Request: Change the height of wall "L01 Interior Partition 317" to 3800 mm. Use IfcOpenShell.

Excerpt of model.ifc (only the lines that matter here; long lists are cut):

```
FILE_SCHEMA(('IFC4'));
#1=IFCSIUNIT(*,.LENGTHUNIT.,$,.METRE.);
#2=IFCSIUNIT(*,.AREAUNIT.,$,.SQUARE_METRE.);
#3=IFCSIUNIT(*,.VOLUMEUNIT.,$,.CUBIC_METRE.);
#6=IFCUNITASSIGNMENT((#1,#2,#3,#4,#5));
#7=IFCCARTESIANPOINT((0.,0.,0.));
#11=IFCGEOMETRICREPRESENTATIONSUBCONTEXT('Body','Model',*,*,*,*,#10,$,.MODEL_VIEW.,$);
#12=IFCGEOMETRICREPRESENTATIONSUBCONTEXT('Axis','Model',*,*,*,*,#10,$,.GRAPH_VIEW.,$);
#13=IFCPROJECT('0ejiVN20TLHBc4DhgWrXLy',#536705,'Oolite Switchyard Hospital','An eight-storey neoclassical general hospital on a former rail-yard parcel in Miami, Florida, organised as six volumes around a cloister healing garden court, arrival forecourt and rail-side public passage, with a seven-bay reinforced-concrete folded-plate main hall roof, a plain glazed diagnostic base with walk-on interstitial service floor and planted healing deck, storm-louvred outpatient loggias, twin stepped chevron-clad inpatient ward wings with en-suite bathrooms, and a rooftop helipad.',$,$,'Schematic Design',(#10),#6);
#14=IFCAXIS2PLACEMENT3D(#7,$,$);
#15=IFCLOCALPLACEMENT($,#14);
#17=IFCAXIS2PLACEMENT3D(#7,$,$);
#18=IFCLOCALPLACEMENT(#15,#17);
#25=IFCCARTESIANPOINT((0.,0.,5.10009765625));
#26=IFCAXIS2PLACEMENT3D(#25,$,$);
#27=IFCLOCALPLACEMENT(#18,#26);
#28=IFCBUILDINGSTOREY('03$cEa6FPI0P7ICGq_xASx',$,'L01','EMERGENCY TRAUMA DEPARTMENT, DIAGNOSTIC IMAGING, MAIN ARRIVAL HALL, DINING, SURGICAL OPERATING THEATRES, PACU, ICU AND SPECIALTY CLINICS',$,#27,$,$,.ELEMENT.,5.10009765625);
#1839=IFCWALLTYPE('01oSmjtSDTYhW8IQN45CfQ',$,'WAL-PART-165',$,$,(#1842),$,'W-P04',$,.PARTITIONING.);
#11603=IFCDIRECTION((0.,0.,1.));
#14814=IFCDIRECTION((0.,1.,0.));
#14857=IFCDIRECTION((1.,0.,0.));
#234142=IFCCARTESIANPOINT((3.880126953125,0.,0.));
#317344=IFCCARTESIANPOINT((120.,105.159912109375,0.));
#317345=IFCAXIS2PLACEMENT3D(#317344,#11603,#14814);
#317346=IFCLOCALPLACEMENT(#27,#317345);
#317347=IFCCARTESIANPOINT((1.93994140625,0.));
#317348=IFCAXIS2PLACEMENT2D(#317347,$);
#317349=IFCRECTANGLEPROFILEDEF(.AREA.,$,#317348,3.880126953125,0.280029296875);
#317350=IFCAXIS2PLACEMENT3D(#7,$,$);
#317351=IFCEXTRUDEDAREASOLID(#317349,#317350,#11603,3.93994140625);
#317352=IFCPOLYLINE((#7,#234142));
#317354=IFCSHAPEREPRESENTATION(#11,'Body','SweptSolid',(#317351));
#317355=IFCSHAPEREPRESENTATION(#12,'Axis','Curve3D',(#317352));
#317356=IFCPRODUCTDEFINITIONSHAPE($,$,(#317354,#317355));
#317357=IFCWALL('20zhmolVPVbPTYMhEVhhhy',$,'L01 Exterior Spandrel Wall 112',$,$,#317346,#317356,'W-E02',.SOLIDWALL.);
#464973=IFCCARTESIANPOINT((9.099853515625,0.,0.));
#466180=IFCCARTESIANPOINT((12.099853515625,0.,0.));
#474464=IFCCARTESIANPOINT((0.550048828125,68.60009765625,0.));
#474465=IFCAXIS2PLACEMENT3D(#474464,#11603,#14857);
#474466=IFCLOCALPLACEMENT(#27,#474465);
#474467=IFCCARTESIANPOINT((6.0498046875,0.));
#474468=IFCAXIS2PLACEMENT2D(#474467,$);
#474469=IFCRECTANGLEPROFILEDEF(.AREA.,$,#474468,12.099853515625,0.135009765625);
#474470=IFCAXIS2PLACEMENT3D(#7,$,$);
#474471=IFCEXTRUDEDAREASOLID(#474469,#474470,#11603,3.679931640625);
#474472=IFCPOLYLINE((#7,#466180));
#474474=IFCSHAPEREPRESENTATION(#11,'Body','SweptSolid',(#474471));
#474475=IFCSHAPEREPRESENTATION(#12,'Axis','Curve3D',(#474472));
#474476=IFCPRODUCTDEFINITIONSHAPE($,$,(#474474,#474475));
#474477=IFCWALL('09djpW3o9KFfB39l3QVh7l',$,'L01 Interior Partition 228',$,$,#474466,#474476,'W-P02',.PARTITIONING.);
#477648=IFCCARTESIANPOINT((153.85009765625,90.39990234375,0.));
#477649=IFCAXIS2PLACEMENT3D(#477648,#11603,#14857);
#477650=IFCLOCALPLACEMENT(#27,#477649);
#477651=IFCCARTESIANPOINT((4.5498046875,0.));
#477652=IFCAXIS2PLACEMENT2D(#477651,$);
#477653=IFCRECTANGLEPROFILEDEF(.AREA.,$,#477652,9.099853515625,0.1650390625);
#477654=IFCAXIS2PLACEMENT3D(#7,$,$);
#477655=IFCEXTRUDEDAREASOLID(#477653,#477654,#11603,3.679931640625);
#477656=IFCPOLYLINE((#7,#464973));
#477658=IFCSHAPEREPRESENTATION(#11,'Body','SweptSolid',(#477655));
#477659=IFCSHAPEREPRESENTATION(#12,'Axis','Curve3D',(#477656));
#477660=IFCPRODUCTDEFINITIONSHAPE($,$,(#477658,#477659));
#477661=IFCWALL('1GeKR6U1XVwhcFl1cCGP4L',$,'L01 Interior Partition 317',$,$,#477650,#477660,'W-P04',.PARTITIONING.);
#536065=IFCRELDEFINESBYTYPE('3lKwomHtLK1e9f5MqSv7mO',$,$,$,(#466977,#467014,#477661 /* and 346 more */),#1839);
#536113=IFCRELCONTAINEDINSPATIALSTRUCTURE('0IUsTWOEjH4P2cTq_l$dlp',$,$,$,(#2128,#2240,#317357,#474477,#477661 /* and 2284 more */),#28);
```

```python
import ifcopenshell
import ifcopenshell.geom
import ifcopenshell.util.representation
import ifcopenshell.util.shape

model = ifcopenshell.open("model.ifc")
settings = ifcopenshell.geom.settings()


def volume(element):
    """Net volume in cubic metres, openings subtracted."""
    shape = ifcopenshell.geom.create_shape(settings, element)
    return ifcopenshell.util.shape.get_volume(shape.geometry)


wall = model.by_guid("1GeKR6U1XVwhcFl1cCGP4L")
before = volume(wall)

body = ifcopenshell.util.representation.get_representation(wall, "Model", "Body")
solid = body.Items[0]
old_height = solid.Depth
solid.Depth = 3.8
after = volume(wall)

print(f"height {old_height:g} -> {solid.Depth:g}, volume {before:.3f} -> {after:.3f} m3")

model.write("model_updated.ifc")
```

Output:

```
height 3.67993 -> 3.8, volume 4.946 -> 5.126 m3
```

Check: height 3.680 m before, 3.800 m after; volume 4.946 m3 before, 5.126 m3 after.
